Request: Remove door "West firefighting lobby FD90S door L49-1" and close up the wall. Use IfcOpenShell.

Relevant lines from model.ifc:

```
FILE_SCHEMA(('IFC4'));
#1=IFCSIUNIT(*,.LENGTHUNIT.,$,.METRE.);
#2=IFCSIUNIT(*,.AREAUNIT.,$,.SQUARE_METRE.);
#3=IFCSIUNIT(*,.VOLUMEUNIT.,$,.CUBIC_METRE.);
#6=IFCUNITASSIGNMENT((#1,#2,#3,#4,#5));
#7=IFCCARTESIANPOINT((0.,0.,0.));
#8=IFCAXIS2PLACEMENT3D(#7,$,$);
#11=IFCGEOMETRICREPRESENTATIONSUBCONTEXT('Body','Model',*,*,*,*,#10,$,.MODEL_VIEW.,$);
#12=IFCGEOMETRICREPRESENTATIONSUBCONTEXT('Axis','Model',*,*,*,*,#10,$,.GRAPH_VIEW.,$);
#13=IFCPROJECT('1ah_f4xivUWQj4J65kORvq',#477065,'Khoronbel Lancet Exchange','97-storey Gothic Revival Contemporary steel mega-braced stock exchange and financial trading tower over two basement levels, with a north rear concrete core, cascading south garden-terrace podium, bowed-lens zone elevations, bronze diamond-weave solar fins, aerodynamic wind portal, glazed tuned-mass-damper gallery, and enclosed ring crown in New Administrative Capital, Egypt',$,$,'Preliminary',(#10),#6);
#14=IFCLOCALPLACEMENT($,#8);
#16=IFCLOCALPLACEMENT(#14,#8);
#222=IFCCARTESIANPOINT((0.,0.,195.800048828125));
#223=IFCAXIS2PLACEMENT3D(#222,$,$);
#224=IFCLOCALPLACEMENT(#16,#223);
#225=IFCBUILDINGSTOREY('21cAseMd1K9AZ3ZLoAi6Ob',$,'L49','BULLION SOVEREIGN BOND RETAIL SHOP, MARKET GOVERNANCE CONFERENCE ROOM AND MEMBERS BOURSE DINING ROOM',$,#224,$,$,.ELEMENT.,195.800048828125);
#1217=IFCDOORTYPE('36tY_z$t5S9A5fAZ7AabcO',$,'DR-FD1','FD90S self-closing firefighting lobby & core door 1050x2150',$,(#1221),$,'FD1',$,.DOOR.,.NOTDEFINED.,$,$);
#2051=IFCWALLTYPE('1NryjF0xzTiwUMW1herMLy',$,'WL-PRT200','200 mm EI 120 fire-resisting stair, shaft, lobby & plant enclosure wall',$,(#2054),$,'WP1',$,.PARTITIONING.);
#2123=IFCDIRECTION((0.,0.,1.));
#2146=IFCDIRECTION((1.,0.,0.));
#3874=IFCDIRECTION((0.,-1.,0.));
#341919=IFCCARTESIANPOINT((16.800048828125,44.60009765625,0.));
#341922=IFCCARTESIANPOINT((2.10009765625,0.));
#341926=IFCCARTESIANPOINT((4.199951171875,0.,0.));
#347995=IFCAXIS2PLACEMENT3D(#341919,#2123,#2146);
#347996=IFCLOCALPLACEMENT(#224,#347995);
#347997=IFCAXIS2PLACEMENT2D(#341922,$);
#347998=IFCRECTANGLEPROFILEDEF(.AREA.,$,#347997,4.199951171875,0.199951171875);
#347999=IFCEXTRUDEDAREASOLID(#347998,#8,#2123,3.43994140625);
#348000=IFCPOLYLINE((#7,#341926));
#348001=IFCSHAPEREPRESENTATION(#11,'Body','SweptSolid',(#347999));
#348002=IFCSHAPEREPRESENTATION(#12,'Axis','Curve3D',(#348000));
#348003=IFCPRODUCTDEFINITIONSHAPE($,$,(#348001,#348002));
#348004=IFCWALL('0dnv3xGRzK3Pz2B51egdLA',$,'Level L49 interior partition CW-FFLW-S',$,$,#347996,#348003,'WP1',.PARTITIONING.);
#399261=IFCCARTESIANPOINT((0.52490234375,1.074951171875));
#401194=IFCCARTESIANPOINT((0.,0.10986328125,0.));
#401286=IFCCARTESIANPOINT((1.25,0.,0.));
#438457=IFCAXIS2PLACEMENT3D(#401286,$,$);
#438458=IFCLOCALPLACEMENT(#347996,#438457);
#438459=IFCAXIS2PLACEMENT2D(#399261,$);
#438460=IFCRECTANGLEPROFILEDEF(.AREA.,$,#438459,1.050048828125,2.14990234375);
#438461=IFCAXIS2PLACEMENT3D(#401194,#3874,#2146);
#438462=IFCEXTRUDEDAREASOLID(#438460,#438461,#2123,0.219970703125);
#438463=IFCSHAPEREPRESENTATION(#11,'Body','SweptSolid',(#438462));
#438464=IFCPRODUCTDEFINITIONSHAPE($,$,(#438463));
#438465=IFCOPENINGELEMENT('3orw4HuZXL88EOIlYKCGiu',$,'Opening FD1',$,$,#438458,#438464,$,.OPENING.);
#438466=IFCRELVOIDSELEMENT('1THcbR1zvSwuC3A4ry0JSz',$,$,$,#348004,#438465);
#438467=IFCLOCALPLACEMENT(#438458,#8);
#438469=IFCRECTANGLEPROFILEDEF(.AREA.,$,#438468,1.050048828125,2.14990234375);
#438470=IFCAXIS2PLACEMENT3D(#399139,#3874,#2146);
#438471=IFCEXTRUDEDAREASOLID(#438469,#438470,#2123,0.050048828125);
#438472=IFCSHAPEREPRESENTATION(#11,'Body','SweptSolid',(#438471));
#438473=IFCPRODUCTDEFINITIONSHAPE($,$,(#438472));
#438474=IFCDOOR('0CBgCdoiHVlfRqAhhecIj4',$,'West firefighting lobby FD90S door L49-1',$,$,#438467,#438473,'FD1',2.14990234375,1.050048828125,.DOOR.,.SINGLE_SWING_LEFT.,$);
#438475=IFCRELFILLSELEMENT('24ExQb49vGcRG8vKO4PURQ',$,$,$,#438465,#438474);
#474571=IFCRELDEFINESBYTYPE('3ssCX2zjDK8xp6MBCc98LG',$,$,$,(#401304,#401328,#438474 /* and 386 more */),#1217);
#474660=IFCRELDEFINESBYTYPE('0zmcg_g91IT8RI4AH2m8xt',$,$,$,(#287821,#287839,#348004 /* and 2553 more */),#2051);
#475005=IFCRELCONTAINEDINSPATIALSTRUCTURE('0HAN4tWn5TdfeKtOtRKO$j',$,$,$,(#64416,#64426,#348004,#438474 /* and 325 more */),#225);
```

```python
import ifcopenshell
import ifcopenshell.api.feature
import ifcopenshell.api.root
import ifcopenshell.geom
import ifcopenshell.util.shape

model = ifcopenshell.open("model.ifc")
settings = ifcopenshell.geom.settings()


def volume(element):
    """Net volume in cubic metres, openings subtracted."""
    shape = ifcopenshell.geom.create_shape(settings, element)
    return ifcopenshell.util.shape.get_volume(shape.geometry)


door = model.by_guid("0CBgCdoiHVlfRqAhhecIj4")
opening = door.FillsVoids[0].RelatingOpeningElement
wall = opening.VoidsElements[0].RelatingBuildingElement
before = volume(wall)

ifcopenshell.api.root.remove_product(model, product=door)
ifcopenshell.api.feature.remove_feature(model, feature=opening)

after = volume(wall)

print(f"wall volume {before:.3f} -> {after:.3f} m3")

model.write("model-out.ifc")
```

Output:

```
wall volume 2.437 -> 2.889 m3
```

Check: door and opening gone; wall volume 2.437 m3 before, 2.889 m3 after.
